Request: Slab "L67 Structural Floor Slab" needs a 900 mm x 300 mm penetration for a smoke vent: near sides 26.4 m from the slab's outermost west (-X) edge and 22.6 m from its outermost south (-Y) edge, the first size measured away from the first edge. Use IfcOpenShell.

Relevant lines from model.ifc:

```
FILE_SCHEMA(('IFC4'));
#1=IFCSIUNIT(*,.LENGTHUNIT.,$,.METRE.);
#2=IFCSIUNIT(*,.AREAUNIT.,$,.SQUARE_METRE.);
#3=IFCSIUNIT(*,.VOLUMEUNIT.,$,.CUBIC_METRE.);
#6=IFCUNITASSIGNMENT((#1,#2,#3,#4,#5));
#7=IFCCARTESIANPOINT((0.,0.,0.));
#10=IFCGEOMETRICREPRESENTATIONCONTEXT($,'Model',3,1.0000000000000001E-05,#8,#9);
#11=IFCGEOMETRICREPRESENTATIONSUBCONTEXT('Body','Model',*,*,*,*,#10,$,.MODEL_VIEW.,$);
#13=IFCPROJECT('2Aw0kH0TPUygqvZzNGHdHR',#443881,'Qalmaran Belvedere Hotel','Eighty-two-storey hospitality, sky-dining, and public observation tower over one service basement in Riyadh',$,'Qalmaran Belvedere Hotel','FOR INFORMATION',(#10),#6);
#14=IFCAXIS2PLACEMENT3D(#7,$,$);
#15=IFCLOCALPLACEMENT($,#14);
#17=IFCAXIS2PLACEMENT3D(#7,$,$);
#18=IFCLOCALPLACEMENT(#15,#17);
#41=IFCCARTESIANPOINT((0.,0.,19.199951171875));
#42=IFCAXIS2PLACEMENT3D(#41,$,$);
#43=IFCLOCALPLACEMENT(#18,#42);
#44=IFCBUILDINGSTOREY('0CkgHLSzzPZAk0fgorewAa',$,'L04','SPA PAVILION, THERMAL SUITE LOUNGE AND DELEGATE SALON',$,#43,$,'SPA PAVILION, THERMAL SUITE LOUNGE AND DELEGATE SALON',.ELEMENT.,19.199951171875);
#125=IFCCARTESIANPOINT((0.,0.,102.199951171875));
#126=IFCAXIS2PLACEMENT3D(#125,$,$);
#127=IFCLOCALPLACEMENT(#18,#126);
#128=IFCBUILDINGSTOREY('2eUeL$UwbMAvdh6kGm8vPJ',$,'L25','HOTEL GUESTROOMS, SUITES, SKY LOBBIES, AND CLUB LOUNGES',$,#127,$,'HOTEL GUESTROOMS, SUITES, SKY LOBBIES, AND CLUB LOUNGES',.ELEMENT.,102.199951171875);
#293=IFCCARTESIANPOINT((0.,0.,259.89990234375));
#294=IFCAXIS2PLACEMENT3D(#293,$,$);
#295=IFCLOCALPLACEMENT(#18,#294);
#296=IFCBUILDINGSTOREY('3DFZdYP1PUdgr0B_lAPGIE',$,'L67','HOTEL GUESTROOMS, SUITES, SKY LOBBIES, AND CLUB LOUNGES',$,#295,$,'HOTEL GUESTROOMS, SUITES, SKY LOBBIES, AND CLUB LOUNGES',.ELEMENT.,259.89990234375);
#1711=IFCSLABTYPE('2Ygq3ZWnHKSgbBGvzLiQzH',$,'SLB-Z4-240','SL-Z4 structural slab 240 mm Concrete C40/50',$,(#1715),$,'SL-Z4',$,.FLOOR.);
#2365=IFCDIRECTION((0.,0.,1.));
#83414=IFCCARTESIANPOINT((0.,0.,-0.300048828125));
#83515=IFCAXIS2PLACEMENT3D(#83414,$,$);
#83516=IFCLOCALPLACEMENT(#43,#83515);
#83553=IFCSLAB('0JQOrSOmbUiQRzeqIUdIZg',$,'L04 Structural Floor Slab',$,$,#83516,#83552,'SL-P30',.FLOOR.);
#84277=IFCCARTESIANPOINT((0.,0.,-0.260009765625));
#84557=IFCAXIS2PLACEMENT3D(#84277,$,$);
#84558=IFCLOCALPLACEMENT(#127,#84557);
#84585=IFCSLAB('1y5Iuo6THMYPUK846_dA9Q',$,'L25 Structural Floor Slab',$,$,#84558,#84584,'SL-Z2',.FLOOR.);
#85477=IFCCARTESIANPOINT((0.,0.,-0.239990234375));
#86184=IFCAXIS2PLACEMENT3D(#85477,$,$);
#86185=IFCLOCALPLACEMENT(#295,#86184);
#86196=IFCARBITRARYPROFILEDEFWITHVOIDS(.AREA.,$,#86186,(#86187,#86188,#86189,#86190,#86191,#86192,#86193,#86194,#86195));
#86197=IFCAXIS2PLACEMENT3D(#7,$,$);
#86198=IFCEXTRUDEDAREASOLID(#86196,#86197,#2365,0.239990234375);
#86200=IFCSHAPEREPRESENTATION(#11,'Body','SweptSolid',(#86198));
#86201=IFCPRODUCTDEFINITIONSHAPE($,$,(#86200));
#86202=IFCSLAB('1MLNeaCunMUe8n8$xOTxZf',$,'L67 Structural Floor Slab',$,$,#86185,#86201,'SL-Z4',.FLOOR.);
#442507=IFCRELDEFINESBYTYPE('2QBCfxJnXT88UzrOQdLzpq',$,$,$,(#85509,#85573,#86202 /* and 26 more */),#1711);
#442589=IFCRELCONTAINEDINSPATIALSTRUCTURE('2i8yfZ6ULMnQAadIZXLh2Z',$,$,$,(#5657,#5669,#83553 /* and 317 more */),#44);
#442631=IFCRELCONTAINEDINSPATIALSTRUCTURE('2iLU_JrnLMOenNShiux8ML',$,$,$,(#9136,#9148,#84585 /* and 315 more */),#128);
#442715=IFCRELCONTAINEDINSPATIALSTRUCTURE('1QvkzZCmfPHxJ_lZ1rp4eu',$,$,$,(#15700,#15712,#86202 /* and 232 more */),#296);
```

```python
import numpy as np
import ifcopenshell
import ifcopenshell.api.feature
import ifcopenshell.api.geometry
import ifcopenshell.api.root
import ifcopenshell.geom
import ifcopenshell.util.placement
import ifcopenshell.util.representation
import ifcopenshell.util.shape
import ifcopenshell.util.unit

model = ifcopenshell.open("model.ifc")
unit_scale = ifcopenshell.util.unit.calculate_unit_scale(model)
settings = ifcopenshell.geom.settings()


def volume(element):
    """Net volume in cubic metres, openings subtracted."""
    shape = ifcopenshell.geom.create_shape(settings, element)
    return ifcopenshell.util.shape.get_volume(shape.geometry)


slab = model.by_id(86202)
before = volume(slab)

# Extent in the slab's own axes, in metres. The edges named are its -X and -Y sides.
slab_shape = ifcopenshell.geom.create_shape(settings, slab)
vertices = ifcopenshell.util.shape.get_vertices(slab_shape.geometry)
x_min, y_min, bottom = vertices.min(axis=0)
top = vertices[:, 2].max()

opening = ifcopenshell.api.root.create_entity(model, ifc_class="IfcOpeningElement", name="Smoke vent opening", predefined_type="OPENING")
context = ifcopenshell.util.representation.get_context(model, "Model", "Body", "MODEL_VIEW")
width, depth = 0.9, 0.3
outline = [(0.0, 0.0), (width, 0.0), (width, depth), (0.0, depth), (0.0, 0.0)]
# Overshoot both faces by 50 mm so the cut is clean.
shape = ifcopenshell.api.geometry.add_slab_representation(
    model, context=context, depth=top - bottom + 0.1, polyline=outline
)
ifcopenshell.api.geometry.assign_representation(model, product=opening, representation=shape)

matrix = ifcopenshell.util.placement.get_local_placement(slab.ObjectPlacement)
matrix[:, 3] = matrix @ np.append(np.array([x_min + 26.4, y_min + 22.6, bottom - 0.05]) / unit_scale, 1.0)
ifcopenshell.api.geometry.edit_object_placement(model, product=opening, matrix=matrix, is_si=False)
ifcopenshell.api.feature.add_feature(model, feature=opening, element=slab)

after = volume(slab)

print(f"slab volume {before:.3f} -> {after:.3f} m3")

model.write("model_rev.ifc")
```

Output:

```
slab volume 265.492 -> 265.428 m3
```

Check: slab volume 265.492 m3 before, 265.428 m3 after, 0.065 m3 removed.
